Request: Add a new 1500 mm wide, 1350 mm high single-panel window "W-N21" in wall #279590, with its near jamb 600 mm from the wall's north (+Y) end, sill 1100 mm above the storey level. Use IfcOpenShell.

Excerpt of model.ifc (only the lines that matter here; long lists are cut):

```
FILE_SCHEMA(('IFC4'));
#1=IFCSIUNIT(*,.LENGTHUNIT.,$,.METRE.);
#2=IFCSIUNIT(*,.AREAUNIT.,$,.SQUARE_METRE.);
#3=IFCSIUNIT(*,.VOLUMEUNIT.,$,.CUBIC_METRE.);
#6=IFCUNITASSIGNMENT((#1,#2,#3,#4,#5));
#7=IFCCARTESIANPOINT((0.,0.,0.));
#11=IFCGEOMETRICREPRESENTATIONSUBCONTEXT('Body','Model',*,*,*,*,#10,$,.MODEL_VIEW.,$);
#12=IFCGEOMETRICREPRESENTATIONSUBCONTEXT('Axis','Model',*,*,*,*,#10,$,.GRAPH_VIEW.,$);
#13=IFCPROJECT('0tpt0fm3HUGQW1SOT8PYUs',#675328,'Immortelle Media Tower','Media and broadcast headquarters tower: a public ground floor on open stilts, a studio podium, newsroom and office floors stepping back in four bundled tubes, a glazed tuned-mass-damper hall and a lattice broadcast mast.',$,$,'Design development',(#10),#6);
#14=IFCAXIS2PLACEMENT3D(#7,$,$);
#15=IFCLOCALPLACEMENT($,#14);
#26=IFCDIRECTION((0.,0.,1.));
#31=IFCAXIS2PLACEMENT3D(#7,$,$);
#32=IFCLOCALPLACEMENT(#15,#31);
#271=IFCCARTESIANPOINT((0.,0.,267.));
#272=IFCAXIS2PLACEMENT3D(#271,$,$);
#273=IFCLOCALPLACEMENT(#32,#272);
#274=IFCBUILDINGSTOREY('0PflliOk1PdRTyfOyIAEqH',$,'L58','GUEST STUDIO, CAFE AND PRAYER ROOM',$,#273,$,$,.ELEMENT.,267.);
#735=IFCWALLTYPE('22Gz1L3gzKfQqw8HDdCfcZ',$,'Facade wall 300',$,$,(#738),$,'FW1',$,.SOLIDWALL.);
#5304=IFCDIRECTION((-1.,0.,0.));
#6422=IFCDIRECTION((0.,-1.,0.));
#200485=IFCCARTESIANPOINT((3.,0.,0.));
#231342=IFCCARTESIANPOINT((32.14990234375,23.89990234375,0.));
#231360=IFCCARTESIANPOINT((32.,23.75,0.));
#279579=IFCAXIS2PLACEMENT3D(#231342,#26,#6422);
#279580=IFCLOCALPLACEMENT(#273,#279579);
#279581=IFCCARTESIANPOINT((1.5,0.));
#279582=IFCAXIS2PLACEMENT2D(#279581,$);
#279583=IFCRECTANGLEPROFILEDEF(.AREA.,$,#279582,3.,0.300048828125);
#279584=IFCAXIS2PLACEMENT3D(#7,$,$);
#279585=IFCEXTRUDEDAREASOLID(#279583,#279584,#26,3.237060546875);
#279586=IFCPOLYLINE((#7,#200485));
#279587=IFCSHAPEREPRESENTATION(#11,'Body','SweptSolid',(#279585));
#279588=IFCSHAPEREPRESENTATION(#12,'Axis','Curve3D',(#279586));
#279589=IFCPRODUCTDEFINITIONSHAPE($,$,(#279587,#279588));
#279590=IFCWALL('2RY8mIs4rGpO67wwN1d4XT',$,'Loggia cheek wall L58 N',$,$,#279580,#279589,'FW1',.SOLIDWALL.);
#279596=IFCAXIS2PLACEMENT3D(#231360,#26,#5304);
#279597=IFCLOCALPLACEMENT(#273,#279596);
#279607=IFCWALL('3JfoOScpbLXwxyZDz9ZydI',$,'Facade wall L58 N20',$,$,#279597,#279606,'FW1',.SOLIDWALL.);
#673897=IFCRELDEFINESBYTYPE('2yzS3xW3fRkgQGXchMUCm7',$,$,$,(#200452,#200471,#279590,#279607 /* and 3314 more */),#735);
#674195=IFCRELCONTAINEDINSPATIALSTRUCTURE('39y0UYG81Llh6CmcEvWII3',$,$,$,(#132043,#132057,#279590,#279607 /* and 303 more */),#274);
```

```python
import numpy as np
import ifcopenshell
import ifcopenshell.api.feature
import ifcopenshell.api.geometry
import ifcopenshell.api.root
import ifcopenshell.api.spatial
import ifcopenshell.geom
import ifcopenshell.util.element
import ifcopenshell.util.placement
import ifcopenshell.util.representation
import ifcopenshell.util.shape
import ifcopenshell.util.unit

model = ifcopenshell.open("model.ifc")
unit_scale = ifcopenshell.util.unit.calculate_unit_scale(model)
settings = ifcopenshell.geom.settings()


def volume(element):
    """Net volume in cubic metres, openings subtracted."""
    shape = ifcopenshell.geom.create_shape(settings, element)
    return ifcopenshell.util.shape.get_volume(shape.geometry)


wall = model.by_guid("2RY8mIs4rGpO67wwN1d4XT")
storey = ifcopenshell.util.element.get_container(wall, ifc_class="IfcBuildingStorey")
context = ifcopenshell.util.representation.get_context(model, "Model", "Body", "MODEL_VIEW")
before = volume(wall)

width, height, from_end, sill = 1.5, 1.35, 0.6, 1.1  # metres

# The wall runs along its own X axis, and the end named is its -X end.
wall_shape = ifcopenshell.geom.create_shape(settings, wall)
x, y, z = ifcopenshell.util.shape.get_vertices(wall_shape.geometry).T
start = x.min() + from_end
face, thickness = float(y.min()), float(y.max() - y.min())
wall_matrix = ifcopenshell.util.placement.get_local_placement(wall.ObjectPlacement)
level = ifcopenshell.util.placement.get_local_placement(storey.ObjectPlacement)[2, 3]


def in_wall(x, y):
    """Placement at x, y metres in the wall's axes, at sill height."""
    matrix = wall_matrix.copy()
    matrix[:, 3] = wall_matrix @ np.array([x / unit_scale, y / unit_scale, 0.0, 1.0])
    matrix[2, 3] = level + sill / unit_scale
    return matrix


# Opening: a box that overshoots both wall faces by 50 mm.
opening = ifcopenshell.api.root.create_entity(model, ifc_class="IfcOpeningElement", predefined_type="OPENING")
box = ifcopenshell.api.geometry.add_wall_representation(
    model, context=context, length=width, height=height, thickness=thickness + 0.1
)
ifcopenshell.api.geometry.assign_representation(model, product=opening, representation=box)
ifcopenshell.api.geometry.edit_object_placement(model, product=opening, matrix=in_wall(start, face - 0.05), is_si=False)
ifcopenshell.api.feature.add_feature(model, feature=opening, element=wall)

window = ifcopenshell.api.root.create_entity(model, ifc_class="IfcWindow", name="W-N21", predefined_type="WINDOW")
window.OverallWidth, window.OverallHeight = width / unit_scale, height / unit_scale
window.PartitioningType = "SINGLE_PANEL"
body = ifcopenshell.api.geometry.add_window_representation(
    model,
    context=context,
    overall_width=window.OverallWidth,
    overall_height=window.OverallHeight,
    partition_type="SINGLE_PANEL",
)
ifcopenshell.api.geometry.assign_representation(model, product=window, representation=body)
ifcopenshell.api.spatial.assign_container(model, products=[window], relating_structure=storey)
ifcopenshell.api.feature.add_filling(model, opening=opening, element=window)

# Centre the window in the wall's thickness.
ifcopenshell.api.geometry.edit_object_placement(model, product=window, matrix=in_wall(start, face), is_si=False)
window_shape = ifcopenshell.geom.create_shape(settings, window)
depth = ifcopenshell.util.shape.get_vertices(window_shape.geometry)[:, 1]
offset = face + thickness / 2 - (depth.min() + depth.max()) / 2
ifcopenshell.api.geometry.edit_object_placement(model, product=window, matrix=in_wall(start, offset), is_si=False)

after = volume(wall)

print(f"wall volume {before:.3f} -> {after:.3f} m3")

model.write("model_edited.ifc")
```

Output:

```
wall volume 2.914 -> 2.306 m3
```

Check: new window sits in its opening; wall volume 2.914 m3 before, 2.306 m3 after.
